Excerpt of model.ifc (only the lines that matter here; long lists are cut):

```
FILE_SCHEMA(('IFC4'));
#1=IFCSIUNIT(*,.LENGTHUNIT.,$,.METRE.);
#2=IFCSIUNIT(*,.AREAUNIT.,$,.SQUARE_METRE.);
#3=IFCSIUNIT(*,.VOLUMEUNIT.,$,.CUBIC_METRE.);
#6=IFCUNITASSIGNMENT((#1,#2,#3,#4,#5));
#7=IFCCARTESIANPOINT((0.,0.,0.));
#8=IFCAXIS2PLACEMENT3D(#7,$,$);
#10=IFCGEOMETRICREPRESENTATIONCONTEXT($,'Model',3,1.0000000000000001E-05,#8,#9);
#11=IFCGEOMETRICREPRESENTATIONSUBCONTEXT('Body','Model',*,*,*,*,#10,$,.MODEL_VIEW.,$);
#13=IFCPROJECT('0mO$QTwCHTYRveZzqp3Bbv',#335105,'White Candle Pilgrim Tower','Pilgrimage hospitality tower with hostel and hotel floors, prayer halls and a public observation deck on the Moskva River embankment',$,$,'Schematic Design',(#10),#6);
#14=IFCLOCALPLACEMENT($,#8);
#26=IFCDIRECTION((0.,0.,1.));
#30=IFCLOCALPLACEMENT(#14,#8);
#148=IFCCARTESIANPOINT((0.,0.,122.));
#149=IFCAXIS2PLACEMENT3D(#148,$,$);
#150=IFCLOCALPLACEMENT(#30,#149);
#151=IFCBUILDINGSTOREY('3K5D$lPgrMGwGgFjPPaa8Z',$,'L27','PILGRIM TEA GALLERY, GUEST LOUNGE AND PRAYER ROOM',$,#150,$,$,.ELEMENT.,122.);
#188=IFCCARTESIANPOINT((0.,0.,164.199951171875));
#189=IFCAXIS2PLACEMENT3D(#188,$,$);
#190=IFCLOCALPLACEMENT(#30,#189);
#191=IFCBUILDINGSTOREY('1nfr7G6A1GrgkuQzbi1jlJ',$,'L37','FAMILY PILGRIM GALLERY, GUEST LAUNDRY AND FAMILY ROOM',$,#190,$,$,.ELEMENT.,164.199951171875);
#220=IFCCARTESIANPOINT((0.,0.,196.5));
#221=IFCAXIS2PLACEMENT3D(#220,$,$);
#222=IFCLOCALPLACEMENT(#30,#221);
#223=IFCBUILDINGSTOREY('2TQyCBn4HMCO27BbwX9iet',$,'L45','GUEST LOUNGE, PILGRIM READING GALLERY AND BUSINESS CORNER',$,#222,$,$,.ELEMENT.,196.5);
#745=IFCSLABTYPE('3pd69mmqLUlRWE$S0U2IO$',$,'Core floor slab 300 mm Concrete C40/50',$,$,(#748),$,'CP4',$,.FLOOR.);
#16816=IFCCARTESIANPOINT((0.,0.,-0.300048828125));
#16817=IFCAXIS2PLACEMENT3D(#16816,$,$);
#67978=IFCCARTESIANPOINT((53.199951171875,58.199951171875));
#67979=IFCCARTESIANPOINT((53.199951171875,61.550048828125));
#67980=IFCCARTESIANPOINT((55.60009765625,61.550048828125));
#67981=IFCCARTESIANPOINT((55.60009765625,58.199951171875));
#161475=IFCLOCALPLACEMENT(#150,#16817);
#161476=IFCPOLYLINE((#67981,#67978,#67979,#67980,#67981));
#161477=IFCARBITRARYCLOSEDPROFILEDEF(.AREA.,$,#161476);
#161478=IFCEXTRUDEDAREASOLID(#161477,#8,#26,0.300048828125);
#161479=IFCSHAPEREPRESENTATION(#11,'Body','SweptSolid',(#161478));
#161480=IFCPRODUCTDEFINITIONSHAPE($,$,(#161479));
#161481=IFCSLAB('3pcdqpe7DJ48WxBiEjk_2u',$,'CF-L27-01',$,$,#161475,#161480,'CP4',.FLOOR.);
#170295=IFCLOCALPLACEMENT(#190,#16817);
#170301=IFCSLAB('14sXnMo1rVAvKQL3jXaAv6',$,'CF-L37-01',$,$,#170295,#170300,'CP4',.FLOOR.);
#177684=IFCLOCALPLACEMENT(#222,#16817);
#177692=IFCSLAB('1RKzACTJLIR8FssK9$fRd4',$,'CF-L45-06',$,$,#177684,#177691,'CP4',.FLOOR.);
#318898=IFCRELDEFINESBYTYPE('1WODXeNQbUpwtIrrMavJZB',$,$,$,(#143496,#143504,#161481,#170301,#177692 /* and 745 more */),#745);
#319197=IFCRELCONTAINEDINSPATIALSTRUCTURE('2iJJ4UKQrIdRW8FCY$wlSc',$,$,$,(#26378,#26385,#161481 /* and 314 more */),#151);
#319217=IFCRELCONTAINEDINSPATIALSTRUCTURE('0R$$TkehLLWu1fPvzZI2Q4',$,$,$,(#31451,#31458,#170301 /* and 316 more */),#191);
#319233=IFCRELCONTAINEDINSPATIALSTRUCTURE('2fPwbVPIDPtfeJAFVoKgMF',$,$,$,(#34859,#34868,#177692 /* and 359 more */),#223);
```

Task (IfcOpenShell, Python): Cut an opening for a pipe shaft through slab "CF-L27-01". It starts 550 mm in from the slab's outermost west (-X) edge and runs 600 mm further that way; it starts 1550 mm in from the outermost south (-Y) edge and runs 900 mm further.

```python
import numpy as np
import ifcopenshell
import ifcopenshell.api.feature
import ifcopenshell.api.geometry
import ifcopenshell.api.root
import ifcopenshell.geom
import ifcopenshell.util.placement
import ifcopenshell.util.representation
import ifcopenshell.util.shape
import ifcopenshell.util.unit

model = ifcopenshell.open("model.ifc")
unit_scale = ifcopenshell.util.unit.calculate_unit_scale(model)
settings = ifcopenshell.geom.settings()


def volume(element):
    """Net volume in cubic metres, openings subtracted."""
    shape = ifcopenshell.geom.create_shape(settings, element)
    return ifcopenshell.util.shape.get_volume(shape.geometry)


slab = model.by_guid("3pcdqpe7DJ48WxBiEjk_2u")
before = volume(slab)

# Extent in the slab's own axes, in metres. The edges named are its -X and -Y sides.
slab_shape = ifcopenshell.geom.create_shape(settings, slab)
vertices = ifcopenshell.util.shape.get_vertices(slab_shape.geometry)
x_min, y_min, bottom = vertices.min(axis=0)
top = vertices[:, 2].max()

opening = ifcopenshell.api.root.create_entity(model, ifc_class="IfcOpeningElement", name="Pipe shaft opening", predefined_type="OPENING")
context = ifcopenshell.util.representation.get_context(model, "Model", "Body", "MODEL_VIEW")
width, depth = 0.6, 0.9
outline = [(0.0, 0.0), (width, 0.0), (width, depth), (0.0, depth), (0.0, 0.0)]
# Overshoot both faces by 50 mm so the cut is clean.
shape = ifcopenshell.api.geometry.add_slab_representation(
    model, context=context, depth=top - bottom + 0.1, polyline=outline
)
ifcopenshell.api.geometry.assign_representation(model, product=opening, representation=shape)

matrix = ifcopenshell.util.placement.get_local_placement(slab.ObjectPlacement)
matrix[:, 3] = matrix @ np.append(np.array([x_min + 0.55, y_min + 1.55, bottom - 0.05]) / unit_scale, 1.0)
ifcopenshell.api.geometry.edit_object_placement(model, product=opening, matrix=matrix, is_si=False)
ifcopenshell.api.feature.add_feature(model, feature=opening, element=slab)

after = volume(slab)

print(f"slab volume {before:.3f} -> {after:.3f} m3")

model.write("model_v2.ifc")
```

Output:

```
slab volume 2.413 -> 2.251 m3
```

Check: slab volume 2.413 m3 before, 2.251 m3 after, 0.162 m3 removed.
